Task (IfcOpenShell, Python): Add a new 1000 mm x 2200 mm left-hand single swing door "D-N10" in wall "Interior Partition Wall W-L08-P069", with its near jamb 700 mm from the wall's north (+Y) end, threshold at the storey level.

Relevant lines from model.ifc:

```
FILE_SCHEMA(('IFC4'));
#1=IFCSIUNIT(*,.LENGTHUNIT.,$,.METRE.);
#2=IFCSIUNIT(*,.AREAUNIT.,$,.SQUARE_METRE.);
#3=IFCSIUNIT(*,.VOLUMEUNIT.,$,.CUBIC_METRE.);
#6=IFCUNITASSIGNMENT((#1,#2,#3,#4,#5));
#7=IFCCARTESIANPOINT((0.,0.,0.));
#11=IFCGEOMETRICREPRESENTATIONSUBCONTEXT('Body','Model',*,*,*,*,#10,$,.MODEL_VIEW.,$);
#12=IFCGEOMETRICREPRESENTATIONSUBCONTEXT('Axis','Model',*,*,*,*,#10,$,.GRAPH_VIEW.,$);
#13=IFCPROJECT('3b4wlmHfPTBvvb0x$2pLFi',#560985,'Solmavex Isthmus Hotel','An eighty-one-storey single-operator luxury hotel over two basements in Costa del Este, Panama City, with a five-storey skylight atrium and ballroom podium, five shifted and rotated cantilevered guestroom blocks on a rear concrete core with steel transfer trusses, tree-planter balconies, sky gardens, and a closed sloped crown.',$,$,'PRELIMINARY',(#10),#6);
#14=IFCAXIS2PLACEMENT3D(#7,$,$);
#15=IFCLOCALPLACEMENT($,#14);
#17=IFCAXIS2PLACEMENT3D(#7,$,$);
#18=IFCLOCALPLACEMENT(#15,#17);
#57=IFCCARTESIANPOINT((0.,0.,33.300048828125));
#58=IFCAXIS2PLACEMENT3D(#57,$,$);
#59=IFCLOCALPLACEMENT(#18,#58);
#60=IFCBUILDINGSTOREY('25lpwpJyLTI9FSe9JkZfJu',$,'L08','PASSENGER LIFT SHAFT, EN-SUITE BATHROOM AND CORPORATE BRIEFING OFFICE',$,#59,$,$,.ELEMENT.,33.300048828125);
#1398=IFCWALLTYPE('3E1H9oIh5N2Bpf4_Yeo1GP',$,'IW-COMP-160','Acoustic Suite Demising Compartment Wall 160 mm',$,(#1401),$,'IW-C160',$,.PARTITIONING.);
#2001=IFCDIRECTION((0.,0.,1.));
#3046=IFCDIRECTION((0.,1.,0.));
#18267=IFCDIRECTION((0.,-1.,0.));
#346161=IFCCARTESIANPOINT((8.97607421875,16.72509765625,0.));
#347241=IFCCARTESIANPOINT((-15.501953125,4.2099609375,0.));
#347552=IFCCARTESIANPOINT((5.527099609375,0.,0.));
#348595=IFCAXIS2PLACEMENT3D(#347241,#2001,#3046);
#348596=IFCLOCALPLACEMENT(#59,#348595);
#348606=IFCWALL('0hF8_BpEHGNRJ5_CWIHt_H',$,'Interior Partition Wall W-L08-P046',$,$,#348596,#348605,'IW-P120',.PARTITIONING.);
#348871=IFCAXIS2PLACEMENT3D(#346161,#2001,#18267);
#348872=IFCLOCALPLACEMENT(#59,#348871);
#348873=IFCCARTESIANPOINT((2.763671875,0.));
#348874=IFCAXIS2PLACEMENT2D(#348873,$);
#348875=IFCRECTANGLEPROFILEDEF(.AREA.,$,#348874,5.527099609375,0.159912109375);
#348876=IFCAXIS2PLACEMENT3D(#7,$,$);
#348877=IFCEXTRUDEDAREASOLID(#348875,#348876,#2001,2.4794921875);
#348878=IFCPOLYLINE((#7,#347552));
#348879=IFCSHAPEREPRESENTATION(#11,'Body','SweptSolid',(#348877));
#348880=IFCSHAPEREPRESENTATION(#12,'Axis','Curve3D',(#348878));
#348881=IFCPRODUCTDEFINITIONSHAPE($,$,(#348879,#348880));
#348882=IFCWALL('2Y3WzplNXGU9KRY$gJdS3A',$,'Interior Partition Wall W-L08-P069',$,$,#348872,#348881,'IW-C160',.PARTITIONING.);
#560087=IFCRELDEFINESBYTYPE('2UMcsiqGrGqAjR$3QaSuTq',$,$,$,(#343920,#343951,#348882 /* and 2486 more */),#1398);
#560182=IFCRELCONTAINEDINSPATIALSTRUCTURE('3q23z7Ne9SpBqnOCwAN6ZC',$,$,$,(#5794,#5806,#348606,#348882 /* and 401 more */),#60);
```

```python
import numpy as np
import ifcopenshell
import ifcopenshell.api.feature
import ifcopenshell.api.geometry
import ifcopenshell.api.root
import ifcopenshell.api.spatial
import ifcopenshell.geom
import ifcopenshell.util.element
import ifcopenshell.util.placement
import ifcopenshell.util.representation
import ifcopenshell.util.shape
import ifcopenshell.util.unit

model = ifcopenshell.open("model.ifc")
unit_scale = ifcopenshell.util.unit.calculate_unit_scale(model)
settings = ifcopenshell.geom.settings()


def volume(element):
    """Net volume in cubic metres, openings subtracted."""
    shape = ifcopenshell.geom.create_shape(settings, element)
    return ifcopenshell.util.shape.get_volume(shape.geometry)


wall = model.by_guid("2Y3WzplNXGU9KRY$gJdS3A")
storey = ifcopenshell.util.element.get_container(wall, ifc_class="IfcBuildingStorey")
context = ifcopenshell.util.representation.get_context(model, "Model", "Body", "MODEL_VIEW")
before = volume(wall)

width, height, from_end, sill = 1, 2.2, 0.7, 0.0  # metres

# The wall runs along its own X axis, and the end named is its -X end.
wall_shape = ifcopenshell.geom.create_shape(settings, wall)
x, y, z = ifcopenshell.util.shape.get_vertices(wall_shape.geometry).T
start = x.min() + from_end
face, thickness = float(y.min()), float(y.max() - y.min())
wall_matrix = ifcopenshell.util.placement.get_local_placement(wall.ObjectPlacement)
level = ifcopenshell.util.placement.get_local_placement(storey.ObjectPlacement)[2, 3]


def in_wall(x, y):
    """Placement at x, y metres in the wall's axes, at sill height."""
    matrix = wall_matrix.copy()
    matrix[:, 3] = wall_matrix @ np.array([x / unit_scale, y / unit_scale, 0.0, 1.0])
    matrix[2, 3] = level + sill / unit_scale
    return matrix


# Opening: a box that overshoots both wall faces by 50 mm.
opening = ifcopenshell.api.root.create_entity(model, ifc_class="IfcOpeningElement", predefined_type="OPENING")
box = ifcopenshell.api.geometry.add_wall_representation(
    model, context=context, length=width, height=height, thickness=thickness + 0.1
)
ifcopenshell.api.geometry.assign_representation(model, product=opening, representation=box)
ifcopenshell.api.geometry.edit_object_placement(model, product=opening, matrix=in_wall(start, face - 0.05), is_si=False)
ifcopenshell.api.feature.add_feature(model, feature=opening, element=wall)

door = ifcopenshell.api.root.create_entity(model, ifc_class="IfcDoor", name="D-N10", predefined_type="DOOR")
door.OverallWidth, door.OverallHeight = width / unit_scale, height / unit_scale
door.OperationType = "SINGLE_SWING_LEFT"
body = ifcopenshell.api.geometry.add_door_representation(
    model,
    context=context,
    overall_width=door.OverallWidth,
    overall_height=door.OverallHeight,
    operation_type="SINGLE_SWING_LEFT",
    lining_properties={"LiningDepth": thickness / unit_scale, "ThresholdDepth": thickness / unit_scale},
)
ifcopenshell.api.geometry.assign_representation(model, product=door, representation=body)
ifcopenshell.api.spatial.assign_container(model, products=[door], relating_structure=storey)
ifcopenshell.api.feature.add_filling(model, opening=opening, element=door)

# The lining spans the wall, so the door starts at the wall face.
ifcopenshell.api.geometry.edit_object_placement(model, product=door, matrix=in_wall(start, face), is_si=False)

after = volume(wall)

print(f"wall volume {before:.3f} -> {after:.3f} m3")

model.write("model_edited.ifc")
```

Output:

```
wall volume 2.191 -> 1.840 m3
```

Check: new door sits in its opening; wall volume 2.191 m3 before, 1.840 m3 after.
